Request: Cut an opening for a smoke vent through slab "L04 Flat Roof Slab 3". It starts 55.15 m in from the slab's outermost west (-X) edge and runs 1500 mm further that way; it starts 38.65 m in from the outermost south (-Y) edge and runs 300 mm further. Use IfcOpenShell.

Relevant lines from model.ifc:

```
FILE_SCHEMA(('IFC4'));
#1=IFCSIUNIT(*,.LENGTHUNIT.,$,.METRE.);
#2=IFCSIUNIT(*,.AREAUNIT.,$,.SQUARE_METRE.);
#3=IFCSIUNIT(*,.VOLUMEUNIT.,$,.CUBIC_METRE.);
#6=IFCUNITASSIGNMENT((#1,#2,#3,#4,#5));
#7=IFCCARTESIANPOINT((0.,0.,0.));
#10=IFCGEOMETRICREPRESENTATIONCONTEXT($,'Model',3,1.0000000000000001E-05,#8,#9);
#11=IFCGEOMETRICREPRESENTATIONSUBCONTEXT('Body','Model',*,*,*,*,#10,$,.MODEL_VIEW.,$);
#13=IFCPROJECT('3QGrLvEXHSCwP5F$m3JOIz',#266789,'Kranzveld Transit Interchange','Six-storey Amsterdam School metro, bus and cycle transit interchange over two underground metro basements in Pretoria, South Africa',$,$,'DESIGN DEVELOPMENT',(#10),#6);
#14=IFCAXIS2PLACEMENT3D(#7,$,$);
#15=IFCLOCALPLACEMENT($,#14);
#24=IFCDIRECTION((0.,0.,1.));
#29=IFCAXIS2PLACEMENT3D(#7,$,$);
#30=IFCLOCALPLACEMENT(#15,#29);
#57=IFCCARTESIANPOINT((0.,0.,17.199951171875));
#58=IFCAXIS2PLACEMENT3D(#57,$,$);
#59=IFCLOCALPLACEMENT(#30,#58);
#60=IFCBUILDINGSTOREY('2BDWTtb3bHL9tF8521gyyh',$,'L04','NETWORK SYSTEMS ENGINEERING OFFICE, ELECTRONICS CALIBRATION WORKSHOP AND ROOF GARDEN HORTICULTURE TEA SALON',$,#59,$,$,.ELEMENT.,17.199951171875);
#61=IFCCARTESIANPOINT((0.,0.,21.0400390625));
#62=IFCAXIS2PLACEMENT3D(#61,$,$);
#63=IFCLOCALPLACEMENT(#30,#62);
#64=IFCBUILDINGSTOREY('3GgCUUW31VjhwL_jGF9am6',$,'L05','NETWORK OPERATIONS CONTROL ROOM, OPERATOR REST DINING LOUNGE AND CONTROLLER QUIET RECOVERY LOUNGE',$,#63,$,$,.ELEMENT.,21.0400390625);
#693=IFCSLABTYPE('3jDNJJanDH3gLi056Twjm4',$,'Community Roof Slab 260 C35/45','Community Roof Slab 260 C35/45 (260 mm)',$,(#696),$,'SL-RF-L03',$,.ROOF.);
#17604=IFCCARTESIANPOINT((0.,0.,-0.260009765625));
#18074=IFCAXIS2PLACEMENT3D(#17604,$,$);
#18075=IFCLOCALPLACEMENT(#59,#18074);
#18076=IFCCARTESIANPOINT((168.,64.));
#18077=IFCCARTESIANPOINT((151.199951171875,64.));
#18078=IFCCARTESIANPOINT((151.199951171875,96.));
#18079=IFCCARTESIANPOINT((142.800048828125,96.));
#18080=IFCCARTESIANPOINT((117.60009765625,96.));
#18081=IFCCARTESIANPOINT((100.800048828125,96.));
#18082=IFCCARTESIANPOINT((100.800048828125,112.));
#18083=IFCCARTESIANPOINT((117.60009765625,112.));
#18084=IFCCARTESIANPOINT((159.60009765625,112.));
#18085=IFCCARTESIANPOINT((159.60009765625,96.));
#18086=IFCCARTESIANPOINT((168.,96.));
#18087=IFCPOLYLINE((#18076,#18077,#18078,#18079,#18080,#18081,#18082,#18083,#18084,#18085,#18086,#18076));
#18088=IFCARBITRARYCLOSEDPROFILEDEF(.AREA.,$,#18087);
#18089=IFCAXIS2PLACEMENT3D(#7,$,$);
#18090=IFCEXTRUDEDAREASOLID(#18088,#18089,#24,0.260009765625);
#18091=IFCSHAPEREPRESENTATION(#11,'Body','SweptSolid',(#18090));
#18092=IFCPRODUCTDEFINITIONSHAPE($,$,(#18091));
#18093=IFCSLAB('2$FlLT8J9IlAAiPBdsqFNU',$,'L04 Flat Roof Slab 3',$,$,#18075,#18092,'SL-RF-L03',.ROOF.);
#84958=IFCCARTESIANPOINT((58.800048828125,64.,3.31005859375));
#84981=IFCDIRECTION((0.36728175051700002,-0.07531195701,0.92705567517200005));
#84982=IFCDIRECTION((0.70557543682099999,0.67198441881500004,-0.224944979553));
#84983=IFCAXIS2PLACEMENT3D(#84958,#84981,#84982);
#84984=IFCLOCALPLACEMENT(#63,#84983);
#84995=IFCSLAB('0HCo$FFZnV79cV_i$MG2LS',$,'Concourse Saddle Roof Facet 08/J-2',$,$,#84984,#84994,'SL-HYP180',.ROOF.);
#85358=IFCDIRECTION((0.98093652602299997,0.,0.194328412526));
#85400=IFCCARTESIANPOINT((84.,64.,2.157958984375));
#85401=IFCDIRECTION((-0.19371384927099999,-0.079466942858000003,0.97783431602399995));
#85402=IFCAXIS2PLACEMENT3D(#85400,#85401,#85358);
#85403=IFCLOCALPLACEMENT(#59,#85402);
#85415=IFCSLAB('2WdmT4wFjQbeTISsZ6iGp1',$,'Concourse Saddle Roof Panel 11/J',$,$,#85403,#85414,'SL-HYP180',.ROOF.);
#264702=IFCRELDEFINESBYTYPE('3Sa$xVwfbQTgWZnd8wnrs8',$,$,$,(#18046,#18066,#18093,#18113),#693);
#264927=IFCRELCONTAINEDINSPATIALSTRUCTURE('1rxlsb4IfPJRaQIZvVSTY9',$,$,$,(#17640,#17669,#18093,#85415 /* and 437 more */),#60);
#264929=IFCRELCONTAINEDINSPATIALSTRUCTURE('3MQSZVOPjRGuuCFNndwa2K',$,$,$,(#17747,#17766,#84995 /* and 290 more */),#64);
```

```python
import numpy as np
import ifcopenshell
import ifcopenshell.api.feature
import ifcopenshell.api.geometry
import ifcopenshell.api.root
import ifcopenshell.geom
import ifcopenshell.util.placement
import ifcopenshell.util.representation
import ifcopenshell.util.shape
import ifcopenshell.util.unit

model = ifcopenshell.open("model.ifc")
unit_scale = ifcopenshell.util.unit.calculate_unit_scale(model)
settings = ifcopenshell.geom.settings()


def volume(element):
    """Net volume in cubic metres, openings subtracted."""
    shape = ifcopenshell.geom.create_shape(settings, element)
    return ifcopenshell.util.shape.get_volume(shape.geometry)


slab = model.by_id(18093)
before = volume(slab)

# Extent in the slab's own axes, in metres. The edges named are its -X and -Y sides.
slab_shape = ifcopenshell.geom.create_shape(settings, slab)
vertices = ifcopenshell.util.shape.get_vertices(slab_shape.geometry)
x_min, y_min, bottom = vertices.min(axis=0)
top = vertices[:, 2].max()

opening = ifcopenshell.api.root.create_entity(model, ifc_class="IfcOpeningElement", name="Smoke vent opening", predefined_type="OPENING")
context = ifcopenshell.util.representation.get_context(model, "Model", "Body", "MODEL_VIEW")
width, depth = 1.5, 0.3
outline = [(0.0, 0.0), (width, 0.0), (width, depth), (0.0, depth), (0.0, 0.0)]
# Overshoot both faces by 50 mm so the cut is clean.
shape = ifcopenshell.api.geometry.add_slab_representation(
    model, context=context, depth=top - bottom + 0.1, polyline=outline
)
ifcopenshell.api.geometry.assign_representation(model, product=opening, representation=shape)

matrix = ifcopenshell.util.placement.get_local_placement(slab.ObjectPlacement)
matrix[:, 3] = matrix @ np.append(np.array([x_min + 55.15, y_min + 38.65, bottom - 0.05]) / unit_scale, 1.0)
ifcopenshell.api.geometry.edit_object_placement(model, product=opening, matrix=matrix, is_si=False)
ifcopenshell.api.feature.add_feature(model, feature=opening, element=slab)

after = volume(slab)

print(f"slab volume {before:.3f} -> {after:.3f} m3")

model.write("model_rev.ifc")
```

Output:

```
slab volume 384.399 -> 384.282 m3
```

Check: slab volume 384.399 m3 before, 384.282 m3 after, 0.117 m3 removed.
